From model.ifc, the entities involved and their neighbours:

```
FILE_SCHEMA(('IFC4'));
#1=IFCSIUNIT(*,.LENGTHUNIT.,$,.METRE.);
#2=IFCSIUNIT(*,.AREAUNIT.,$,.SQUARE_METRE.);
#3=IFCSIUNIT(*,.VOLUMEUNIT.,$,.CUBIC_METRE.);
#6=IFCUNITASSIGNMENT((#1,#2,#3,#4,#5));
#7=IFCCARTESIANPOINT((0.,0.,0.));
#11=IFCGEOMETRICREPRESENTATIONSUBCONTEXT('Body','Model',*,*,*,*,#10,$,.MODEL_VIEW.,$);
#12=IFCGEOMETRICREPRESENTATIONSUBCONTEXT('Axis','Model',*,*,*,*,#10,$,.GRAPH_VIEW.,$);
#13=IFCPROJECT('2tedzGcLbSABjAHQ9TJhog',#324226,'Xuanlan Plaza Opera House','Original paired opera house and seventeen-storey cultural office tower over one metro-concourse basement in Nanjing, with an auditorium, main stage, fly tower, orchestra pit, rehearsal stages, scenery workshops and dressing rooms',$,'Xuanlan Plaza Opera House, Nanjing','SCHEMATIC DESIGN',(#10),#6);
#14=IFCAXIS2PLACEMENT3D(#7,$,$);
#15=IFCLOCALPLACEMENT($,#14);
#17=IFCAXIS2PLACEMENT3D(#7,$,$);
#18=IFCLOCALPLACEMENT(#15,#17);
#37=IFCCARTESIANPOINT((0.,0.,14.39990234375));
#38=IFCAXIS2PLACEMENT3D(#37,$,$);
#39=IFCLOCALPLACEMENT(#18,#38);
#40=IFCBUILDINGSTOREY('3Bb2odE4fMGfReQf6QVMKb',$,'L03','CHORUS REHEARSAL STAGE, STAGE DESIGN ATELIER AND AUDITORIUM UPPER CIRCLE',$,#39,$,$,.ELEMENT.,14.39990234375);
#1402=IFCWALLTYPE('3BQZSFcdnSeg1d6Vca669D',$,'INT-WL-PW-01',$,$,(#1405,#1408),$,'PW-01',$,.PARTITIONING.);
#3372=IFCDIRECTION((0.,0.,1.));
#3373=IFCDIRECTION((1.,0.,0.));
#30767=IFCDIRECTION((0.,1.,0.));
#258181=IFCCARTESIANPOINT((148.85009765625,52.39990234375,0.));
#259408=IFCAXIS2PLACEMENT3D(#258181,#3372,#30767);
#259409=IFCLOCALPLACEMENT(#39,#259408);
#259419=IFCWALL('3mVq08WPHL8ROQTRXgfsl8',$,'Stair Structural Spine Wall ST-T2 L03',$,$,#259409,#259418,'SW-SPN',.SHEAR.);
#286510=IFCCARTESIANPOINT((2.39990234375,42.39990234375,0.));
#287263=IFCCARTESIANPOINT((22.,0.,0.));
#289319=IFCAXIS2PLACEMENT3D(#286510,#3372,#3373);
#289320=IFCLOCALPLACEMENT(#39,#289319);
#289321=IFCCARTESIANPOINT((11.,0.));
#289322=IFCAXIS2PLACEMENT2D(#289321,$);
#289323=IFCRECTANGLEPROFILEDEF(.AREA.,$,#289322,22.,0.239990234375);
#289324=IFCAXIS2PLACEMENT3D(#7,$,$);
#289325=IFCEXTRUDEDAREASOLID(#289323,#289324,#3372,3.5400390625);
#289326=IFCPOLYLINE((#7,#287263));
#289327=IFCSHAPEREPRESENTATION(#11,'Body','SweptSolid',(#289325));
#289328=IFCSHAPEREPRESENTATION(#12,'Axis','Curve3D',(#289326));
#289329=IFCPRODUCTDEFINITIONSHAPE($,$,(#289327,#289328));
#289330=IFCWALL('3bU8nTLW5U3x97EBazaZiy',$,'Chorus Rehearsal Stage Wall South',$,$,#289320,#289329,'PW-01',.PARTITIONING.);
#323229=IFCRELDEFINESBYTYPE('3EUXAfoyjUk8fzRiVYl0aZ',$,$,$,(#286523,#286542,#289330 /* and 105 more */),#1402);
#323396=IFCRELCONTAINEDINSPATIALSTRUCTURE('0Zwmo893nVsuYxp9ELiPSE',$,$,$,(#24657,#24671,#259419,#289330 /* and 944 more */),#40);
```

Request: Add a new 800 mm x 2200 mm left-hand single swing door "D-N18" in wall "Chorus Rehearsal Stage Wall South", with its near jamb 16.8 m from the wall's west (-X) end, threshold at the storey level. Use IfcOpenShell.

```python
import numpy as np
import ifcopenshell
import ifcopenshell.api.feature
import ifcopenshell.api.geometry
import ifcopenshell.api.root
import ifcopenshell.api.spatial
import ifcopenshell.geom
import ifcopenshell.util.element
import ifcopenshell.util.placement
import ifcopenshell.util.representation
import ifcopenshell.util.shape
import ifcopenshell.util.unit

model = ifcopenshell.open("model.ifc")
unit_scale = ifcopenshell.util.unit.calculate_unit_scale(model)
settings = ifcopenshell.geom.settings()


def volume(element):
    """Net volume in cubic metres, openings subtracted."""
    shape = ifcopenshell.geom.create_shape(settings, element)
    return ifcopenshell.util.shape.get_volume(shape.geometry)


wall = model.by_id(289330)
storey = ifcopenshell.util.element.get_container(wall, ifc_class="IfcBuildingStorey")
context = ifcopenshell.util.representation.get_context(model, "Model", "Body", "MODEL_VIEW")
before = volume(wall)

width, height, from_end, sill = 0.8, 2.2, 16.8, 0.0  # metres

# The wall runs along its own X axis, and the end named is its -X end.
wall_shape = ifcopenshell.geom.create_shape(settings, wall)
x, y, z = ifcopenshell.util.shape.get_vertices(wall_shape.geometry).T
start = x.min() + from_end
face, thickness = float(y.min()), float(y.max() - y.min())
wall_matrix = ifcopenshell.util.placement.get_local_placement(wall.ObjectPlacement)
level = ifcopenshell.util.placement.get_local_placement(storey.ObjectPlacement)[2, 3]


def in_wall(x, y):
    """Placement at x, y metres in the wall's axes, at sill height."""
    matrix = wall_matrix.copy()
    matrix[:, 3] = wall_matrix @ np.array([x / unit_scale, y / unit_scale, 0.0, 1.0])
    matrix[2, 3] = level + sill / unit_scale
    return matrix


# Opening: a box that overshoots both wall faces by 50 mm.
opening = ifcopenshell.api.root.create_entity(model, ifc_class="IfcOpeningElement", predefined_type="OPENING")
box = ifcopenshell.api.geometry.add_wall_representation(
    model, context=context, length=width, height=height, thickness=thickness + 0.1
)
ifcopenshell.api.geometry.assign_representation(model, product=opening, representation=box)
ifcopenshell.api.geometry.edit_object_placement(model, product=opening, matrix=in_wall(start, face - 0.05), is_si=False)
ifcopenshell.api.feature.add_feature(model, feature=opening, element=wall)

door = ifcopenshell.api.root.create_entity(model, ifc_class="IfcDoor", name="D-N18", predefined_type="DOOR")
door.OverallWidth, door.OverallHeight = width / unit_scale, height / unit_scale
door.OperationType = "SINGLE_SWING_LEFT"
body = ifcopenshell.api.geometry.add_door_representation(
    model,
    context=context,
    overall_width=door.OverallWidth,
    overall_height=door.OverallHeight,
    operation_type="SINGLE_SWING_LEFT",
    lining_properties={"LiningDepth": thickness / unit_scale, "ThresholdDepth": thickness / unit_scale},
)
ifcopenshell.api.geometry.assign_representation(model, product=door, representation=body)
ifcopenshell.api.spatial.assign_container(model, products=[door], relating_structure=storey)
ifcopenshell.api.feature.add_filling(model, opening=opening, element=door)

# The lining spans the wall, so the door starts at the wall face.
ifcopenshell.api.geometry.edit_object_placement(model, product=door, matrix=in_wall(start, face), is_si=False)

after = volume(wall)

print(f"wall volume {before:.3f} -> {after:.3f} m3")

model.write("model-out.ifc")
```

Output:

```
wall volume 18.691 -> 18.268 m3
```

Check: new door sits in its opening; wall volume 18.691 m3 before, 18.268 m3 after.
